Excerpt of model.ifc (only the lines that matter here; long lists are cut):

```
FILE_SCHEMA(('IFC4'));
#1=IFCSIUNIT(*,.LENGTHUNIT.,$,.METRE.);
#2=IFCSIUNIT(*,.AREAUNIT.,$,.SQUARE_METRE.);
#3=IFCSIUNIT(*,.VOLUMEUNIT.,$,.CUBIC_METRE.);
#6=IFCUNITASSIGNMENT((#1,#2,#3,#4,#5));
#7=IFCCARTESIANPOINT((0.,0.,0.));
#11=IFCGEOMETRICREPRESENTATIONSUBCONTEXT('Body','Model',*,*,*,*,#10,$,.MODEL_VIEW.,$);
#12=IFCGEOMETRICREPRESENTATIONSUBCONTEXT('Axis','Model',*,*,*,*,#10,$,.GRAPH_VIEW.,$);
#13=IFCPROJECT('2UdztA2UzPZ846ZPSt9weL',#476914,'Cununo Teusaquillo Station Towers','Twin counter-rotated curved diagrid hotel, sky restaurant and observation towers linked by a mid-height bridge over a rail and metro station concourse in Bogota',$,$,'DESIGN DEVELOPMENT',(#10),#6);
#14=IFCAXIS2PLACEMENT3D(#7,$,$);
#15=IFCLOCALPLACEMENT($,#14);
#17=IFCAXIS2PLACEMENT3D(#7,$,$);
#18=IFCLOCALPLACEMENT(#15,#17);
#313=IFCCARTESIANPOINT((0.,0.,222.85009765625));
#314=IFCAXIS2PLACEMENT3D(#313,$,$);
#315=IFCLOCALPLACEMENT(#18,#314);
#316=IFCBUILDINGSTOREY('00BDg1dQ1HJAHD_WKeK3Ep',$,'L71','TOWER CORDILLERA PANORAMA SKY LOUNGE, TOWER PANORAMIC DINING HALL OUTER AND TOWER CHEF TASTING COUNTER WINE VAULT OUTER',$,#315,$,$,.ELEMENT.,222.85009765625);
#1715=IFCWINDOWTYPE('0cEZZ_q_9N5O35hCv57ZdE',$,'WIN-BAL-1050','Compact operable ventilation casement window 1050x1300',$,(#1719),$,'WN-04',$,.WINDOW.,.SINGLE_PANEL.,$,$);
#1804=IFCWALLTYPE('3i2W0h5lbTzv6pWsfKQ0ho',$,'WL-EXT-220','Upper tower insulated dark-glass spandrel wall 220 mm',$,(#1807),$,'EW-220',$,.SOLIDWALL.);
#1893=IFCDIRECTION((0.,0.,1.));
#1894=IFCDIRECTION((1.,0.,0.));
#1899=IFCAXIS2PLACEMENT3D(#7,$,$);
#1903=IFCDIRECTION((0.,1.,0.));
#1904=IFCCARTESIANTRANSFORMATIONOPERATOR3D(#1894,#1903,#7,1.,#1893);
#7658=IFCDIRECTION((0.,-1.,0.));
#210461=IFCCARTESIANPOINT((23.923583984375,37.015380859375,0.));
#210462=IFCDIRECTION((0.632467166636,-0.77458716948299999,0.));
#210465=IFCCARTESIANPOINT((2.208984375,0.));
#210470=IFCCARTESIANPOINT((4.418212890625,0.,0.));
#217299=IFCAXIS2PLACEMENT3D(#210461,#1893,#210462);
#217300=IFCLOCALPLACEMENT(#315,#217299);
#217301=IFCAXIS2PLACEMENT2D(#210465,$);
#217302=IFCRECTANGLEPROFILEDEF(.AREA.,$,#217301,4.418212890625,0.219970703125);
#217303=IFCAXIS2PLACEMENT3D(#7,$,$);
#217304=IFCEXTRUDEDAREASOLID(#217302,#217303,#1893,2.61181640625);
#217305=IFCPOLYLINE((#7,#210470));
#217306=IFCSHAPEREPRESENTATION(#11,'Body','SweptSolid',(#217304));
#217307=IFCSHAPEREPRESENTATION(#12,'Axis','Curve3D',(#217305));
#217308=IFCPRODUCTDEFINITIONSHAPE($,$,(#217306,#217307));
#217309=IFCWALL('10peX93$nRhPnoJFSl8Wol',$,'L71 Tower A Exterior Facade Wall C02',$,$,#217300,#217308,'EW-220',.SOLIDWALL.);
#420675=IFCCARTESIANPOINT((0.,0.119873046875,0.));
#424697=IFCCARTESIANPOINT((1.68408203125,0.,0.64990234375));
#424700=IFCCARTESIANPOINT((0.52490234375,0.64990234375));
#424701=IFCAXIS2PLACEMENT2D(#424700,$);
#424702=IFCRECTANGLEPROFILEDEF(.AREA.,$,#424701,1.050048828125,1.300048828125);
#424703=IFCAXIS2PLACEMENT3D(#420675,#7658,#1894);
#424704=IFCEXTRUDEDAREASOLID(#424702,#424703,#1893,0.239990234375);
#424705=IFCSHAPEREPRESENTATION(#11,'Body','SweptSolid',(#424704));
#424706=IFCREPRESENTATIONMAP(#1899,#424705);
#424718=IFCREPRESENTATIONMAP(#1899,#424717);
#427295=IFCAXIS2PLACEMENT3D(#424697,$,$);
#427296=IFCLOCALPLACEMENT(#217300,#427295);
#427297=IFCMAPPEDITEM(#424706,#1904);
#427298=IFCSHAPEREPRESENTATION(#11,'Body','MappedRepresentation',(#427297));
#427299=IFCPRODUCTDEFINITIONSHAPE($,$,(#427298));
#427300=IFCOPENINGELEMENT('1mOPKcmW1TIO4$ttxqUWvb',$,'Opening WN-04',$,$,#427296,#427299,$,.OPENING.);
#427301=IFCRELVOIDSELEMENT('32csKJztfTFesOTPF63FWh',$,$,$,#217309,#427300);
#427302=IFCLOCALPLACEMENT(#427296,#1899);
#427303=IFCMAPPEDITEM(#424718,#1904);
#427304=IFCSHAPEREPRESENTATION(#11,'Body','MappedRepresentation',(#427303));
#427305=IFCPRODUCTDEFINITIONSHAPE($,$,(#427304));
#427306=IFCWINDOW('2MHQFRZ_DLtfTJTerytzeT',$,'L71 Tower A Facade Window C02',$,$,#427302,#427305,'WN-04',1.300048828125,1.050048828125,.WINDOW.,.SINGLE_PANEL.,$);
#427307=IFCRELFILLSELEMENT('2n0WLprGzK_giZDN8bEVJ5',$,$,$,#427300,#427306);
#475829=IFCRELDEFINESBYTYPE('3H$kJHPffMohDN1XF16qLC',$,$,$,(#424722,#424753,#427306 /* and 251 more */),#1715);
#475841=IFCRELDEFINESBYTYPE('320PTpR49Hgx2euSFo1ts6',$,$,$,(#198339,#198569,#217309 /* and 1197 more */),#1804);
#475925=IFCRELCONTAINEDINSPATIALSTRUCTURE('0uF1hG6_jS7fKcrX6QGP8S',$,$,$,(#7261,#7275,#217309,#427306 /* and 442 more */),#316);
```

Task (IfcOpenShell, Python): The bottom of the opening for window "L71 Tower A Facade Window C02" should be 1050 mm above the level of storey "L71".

```python
import numpy as np
import ifcopenshell
import ifcopenshell.api.geometry
import ifcopenshell.geom
import ifcopenshell.util.element
import ifcopenshell.util.placement
import ifcopenshell.util.shape
import ifcopenshell.util.unit

model = ifcopenshell.open("model.ifc")
unit_scale = ifcopenshell.util.unit.calculate_unit_scale(model)

window = model.by_guid("2MHQFRZ_DLtfTJTerytzeT")
opening = window.FillsVoids[0].RelatingOpeningElement
storey = ifcopenshell.util.element.get_container(window, ifc_class="IfcBuildingStorey")
level = ifcopenshell.util.placement.get_local_placement(storey.ObjectPlacement)[2, 3]

# The opening's origin need not be at the sill, so measure its lowest point.
shape = ifcopenshell.geom.create_shape(ifcopenshell.geom.settings(), opening)
bottom = ifcopenshell.util.shape.get_shape_bottom_elevation(shape, shape.geometry) / unit_scale
dz = level + 1.05 / unit_scale - bottom

shift = np.array([0.0, 0.0, dz])
# The window is placed relative to its opening, so it follows when the opening moves.
matrix = ifcopenshell.util.placement.get_local_placement(opening.ObjectPlacement)
matrix[:3, 3] += shift
ifcopenshell.api.geometry.edit_object_placement(
    model, product=opening, matrix=matrix, is_si=False, should_transform_children=True
)

print(f"moved by {dz * unit_scale:+.3f} m")

model.write("model_updated.ifc")
```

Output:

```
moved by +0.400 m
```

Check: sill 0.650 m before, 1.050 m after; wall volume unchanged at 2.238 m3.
